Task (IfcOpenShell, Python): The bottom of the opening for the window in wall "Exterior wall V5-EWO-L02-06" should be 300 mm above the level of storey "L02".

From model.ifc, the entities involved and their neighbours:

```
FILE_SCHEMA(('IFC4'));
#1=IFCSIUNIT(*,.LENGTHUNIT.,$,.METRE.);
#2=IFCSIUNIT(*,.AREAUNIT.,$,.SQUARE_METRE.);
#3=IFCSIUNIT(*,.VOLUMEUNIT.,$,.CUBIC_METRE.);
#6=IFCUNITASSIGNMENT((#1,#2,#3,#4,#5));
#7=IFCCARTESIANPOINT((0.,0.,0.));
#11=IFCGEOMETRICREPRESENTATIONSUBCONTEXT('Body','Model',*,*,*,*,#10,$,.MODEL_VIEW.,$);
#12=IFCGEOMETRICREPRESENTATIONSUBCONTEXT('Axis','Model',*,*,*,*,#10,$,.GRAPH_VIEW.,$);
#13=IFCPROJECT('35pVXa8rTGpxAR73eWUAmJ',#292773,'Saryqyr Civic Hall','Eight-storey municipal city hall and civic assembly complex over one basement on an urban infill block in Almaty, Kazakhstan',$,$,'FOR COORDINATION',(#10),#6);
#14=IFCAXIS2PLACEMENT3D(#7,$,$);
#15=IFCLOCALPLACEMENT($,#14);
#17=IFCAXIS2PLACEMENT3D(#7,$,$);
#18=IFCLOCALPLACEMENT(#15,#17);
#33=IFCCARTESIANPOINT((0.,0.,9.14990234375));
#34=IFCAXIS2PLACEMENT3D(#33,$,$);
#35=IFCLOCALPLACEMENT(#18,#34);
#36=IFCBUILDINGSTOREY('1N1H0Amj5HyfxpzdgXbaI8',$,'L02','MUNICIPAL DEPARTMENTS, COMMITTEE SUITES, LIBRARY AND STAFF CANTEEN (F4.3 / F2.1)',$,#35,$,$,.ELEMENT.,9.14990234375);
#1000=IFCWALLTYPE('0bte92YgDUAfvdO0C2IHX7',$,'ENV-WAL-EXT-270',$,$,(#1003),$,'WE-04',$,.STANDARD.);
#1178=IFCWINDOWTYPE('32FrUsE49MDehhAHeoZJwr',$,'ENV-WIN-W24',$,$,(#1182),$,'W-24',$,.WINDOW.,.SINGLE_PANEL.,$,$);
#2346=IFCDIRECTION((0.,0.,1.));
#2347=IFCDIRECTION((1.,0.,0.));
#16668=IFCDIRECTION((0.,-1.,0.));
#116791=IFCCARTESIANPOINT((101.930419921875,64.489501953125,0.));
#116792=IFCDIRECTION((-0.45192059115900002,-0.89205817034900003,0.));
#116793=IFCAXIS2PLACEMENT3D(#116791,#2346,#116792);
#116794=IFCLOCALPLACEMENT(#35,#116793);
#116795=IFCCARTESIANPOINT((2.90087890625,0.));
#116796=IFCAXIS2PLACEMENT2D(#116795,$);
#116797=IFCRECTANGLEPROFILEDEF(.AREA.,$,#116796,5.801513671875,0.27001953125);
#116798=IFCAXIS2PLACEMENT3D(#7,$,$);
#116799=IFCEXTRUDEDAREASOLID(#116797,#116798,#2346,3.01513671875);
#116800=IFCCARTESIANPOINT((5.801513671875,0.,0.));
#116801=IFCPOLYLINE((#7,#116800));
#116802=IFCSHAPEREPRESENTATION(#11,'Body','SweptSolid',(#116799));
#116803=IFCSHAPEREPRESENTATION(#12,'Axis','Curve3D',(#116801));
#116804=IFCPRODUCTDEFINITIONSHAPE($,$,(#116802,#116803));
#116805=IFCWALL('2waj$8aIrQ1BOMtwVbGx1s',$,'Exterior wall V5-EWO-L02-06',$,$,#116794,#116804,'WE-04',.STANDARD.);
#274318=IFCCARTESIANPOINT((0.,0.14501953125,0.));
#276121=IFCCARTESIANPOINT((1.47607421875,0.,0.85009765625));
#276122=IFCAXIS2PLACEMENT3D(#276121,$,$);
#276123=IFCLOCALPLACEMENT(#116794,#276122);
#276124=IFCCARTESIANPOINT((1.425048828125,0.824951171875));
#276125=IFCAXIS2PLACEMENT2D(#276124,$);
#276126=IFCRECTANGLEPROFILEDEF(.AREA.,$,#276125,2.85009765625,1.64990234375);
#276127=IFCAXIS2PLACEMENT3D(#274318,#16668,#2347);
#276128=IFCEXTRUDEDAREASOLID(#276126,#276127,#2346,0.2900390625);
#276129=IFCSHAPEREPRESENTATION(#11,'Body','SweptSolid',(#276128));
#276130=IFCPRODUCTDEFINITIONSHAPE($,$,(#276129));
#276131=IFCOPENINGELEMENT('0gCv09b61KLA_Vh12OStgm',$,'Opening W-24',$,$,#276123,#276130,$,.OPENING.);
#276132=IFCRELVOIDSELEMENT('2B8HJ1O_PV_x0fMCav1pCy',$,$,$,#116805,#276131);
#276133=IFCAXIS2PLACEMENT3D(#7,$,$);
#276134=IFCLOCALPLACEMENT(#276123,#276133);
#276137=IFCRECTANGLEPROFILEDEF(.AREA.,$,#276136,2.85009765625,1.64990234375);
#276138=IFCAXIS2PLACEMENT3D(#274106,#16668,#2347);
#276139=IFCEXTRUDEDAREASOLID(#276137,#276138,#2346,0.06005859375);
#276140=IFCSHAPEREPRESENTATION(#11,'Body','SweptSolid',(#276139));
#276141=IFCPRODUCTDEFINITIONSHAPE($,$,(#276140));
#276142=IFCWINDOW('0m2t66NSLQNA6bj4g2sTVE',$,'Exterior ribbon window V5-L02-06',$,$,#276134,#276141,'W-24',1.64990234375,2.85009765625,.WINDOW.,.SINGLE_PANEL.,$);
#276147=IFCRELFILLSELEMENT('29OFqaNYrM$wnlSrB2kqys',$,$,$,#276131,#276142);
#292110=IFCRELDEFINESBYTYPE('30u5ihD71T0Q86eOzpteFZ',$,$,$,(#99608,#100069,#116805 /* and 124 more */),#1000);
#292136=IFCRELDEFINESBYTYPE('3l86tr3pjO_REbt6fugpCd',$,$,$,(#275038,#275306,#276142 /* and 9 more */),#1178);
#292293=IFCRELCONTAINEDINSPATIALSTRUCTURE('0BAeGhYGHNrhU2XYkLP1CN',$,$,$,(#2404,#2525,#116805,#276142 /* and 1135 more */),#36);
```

```python
import numpy as np
import ifcopenshell
import ifcopenshell.api.geometry
import ifcopenshell.geom
import ifcopenshell.util.element
import ifcopenshell.util.placement
import ifcopenshell.util.shape
import ifcopenshell.util.unit

model = ifcopenshell.open("model.ifc")
unit_scale = ifcopenshell.util.unit.calculate_unit_scale(model)

window = model.by_guid("0m2t66NSLQNA6bj4g2sTVE")
opening = window.FillsVoids[0].RelatingOpeningElement
storey = ifcopenshell.util.element.get_container(window, ifc_class="IfcBuildingStorey")
level = ifcopenshell.util.placement.get_local_placement(storey.ObjectPlacement)[2, 3]

# The opening's origin need not be at the sill, so measure its lowest point.
shape = ifcopenshell.geom.create_shape(ifcopenshell.geom.settings(), opening)
bottom = ifcopenshell.util.shape.get_shape_bottom_elevation(shape, shape.geometry) / unit_scale
dz = level + 0.3 / unit_scale - bottom

shift = np.array([0.0, 0.0, dz])
# The window is placed relative to its opening, so it follows when the opening moves.
matrix = ifcopenshell.util.placement.get_local_placement(opening.ObjectPlacement)
matrix[:3, 3] += shift
ifcopenshell.api.geometry.edit_object_placement(
    model, product=opening, matrix=matrix, is_si=False, should_transform_children=True
)

print(f"moved by {dz * unit_scale:+.3f} m")

model.write("model-out.ifc")
```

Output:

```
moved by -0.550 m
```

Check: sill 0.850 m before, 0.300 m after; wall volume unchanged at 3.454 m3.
